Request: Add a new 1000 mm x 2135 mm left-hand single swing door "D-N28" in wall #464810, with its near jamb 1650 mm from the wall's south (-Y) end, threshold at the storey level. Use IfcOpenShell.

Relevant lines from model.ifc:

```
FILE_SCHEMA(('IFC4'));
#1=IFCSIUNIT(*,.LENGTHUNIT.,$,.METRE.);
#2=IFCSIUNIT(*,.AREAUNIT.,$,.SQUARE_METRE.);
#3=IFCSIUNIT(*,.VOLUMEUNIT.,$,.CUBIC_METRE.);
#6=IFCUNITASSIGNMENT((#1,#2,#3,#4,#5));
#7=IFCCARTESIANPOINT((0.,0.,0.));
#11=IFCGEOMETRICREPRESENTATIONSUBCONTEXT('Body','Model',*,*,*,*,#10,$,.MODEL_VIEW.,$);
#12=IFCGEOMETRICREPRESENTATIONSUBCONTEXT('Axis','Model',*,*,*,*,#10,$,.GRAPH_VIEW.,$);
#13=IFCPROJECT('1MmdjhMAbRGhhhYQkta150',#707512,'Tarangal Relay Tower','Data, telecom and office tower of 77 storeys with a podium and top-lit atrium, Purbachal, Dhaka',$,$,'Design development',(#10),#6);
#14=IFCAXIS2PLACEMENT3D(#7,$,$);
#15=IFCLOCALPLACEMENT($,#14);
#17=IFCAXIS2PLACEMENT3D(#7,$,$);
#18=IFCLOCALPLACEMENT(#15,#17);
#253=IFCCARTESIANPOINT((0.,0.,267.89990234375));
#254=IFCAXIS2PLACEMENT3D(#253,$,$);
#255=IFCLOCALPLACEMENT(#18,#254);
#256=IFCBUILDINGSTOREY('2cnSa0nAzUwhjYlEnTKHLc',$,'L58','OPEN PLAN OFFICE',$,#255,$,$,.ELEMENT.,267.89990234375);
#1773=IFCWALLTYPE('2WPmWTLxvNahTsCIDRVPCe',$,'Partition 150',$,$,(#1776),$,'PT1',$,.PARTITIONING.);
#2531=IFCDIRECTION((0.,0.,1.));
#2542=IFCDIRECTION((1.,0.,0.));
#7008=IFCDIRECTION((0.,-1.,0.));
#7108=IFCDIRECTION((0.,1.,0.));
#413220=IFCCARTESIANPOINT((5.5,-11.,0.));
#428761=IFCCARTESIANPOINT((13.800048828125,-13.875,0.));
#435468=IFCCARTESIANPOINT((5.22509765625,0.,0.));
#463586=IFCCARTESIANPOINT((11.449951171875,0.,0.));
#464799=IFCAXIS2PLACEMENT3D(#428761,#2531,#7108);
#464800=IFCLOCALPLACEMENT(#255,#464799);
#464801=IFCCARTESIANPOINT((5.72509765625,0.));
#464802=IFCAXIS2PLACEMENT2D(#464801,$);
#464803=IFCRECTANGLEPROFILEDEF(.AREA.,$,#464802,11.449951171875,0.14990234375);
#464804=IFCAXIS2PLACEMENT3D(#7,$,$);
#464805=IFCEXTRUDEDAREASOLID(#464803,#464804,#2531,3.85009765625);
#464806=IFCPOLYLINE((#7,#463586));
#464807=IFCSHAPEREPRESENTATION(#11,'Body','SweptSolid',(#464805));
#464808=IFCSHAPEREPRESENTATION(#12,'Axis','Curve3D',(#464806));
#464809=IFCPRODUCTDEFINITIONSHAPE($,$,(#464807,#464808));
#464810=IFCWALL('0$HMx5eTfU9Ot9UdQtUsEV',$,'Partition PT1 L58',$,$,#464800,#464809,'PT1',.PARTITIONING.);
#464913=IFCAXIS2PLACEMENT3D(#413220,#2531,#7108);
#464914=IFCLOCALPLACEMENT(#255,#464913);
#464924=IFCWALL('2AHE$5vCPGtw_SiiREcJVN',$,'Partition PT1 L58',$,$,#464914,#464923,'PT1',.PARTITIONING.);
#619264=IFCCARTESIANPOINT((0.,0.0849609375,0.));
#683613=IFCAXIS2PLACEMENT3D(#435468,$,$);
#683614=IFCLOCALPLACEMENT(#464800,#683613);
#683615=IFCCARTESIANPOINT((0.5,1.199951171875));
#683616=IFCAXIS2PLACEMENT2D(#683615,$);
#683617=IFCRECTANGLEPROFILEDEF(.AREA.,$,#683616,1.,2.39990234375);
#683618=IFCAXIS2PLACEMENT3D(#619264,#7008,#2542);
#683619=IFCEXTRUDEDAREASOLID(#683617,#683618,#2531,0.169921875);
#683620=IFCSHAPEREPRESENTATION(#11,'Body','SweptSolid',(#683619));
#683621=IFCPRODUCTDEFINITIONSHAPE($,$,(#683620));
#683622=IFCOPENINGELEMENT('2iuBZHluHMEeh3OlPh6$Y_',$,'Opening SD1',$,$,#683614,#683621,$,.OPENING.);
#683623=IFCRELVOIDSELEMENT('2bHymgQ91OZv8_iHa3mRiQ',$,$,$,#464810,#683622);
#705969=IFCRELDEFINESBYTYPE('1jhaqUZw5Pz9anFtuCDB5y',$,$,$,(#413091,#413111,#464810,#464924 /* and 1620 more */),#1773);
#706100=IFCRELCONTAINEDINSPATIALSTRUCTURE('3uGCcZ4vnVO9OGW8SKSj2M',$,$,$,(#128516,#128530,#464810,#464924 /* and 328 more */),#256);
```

```python
import numpy as np
import ifcopenshell
import ifcopenshell.api.feature
import ifcopenshell.api.geometry
import ifcopenshell.api.root
import ifcopenshell.api.spatial
import ifcopenshell.geom
import ifcopenshell.util.element
import ifcopenshell.util.placement
import ifcopenshell.util.representation
import ifcopenshell.util.shape
import ifcopenshell.util.unit

model = ifcopenshell.open("model.ifc")
unit_scale = ifcopenshell.util.unit.calculate_unit_scale(model)
settings = ifcopenshell.geom.settings()


def volume(element):
    """Net volume in cubic metres, openings subtracted."""
    shape = ifcopenshell.geom.create_shape(settings, element)
    return ifcopenshell.util.shape.get_volume(shape.geometry)


wall = model.by_id(464810)
storey = ifcopenshell.util.element.get_container(wall, ifc_class="IfcBuildingStorey")
context = ifcopenshell.util.representation.get_context(model, "Model", "Body", "MODEL_VIEW")
before = volume(wall)

width, height, from_end, sill = 1, 2.135, 1.65, 0.0  # metres

# The wall runs along its own X axis, and the end named is its -X end.
wall_shape = ifcopenshell.geom.create_shape(settings, wall)
x, y, z = ifcopenshell.util.shape.get_vertices(wall_shape.geometry).T
start = x.min() + from_end
face, thickness = float(y.min()), float(y.max() - y.min())
wall_matrix = ifcopenshell.util.placement.get_local_placement(wall.ObjectPlacement)
level = ifcopenshell.util.placement.get_local_placement(storey.ObjectPlacement)[2, 3]


def in_wall(x, y):
    """Placement at x, y metres in the wall's axes, at sill height."""
    matrix = wall_matrix.copy()
    matrix[:, 3] = wall_matrix @ np.array([x / unit_scale, y / unit_scale, 0.0, 1.0])
    matrix[2, 3] = level + sill / unit_scale
    return matrix


# Opening: a box that overshoots both wall faces by 50 mm.
opening = ifcopenshell.api.root.create_entity(model, ifc_class="IfcOpeningElement", predefined_type="OPENING")
box = ifcopenshell.api.geometry.add_wall_representation(
    model, context=context, length=width, height=height, thickness=thickness + 0.1
)
ifcopenshell.api.geometry.assign_representation(model, product=opening, representation=box)
ifcopenshell.api.geometry.edit_object_placement(model, product=opening, matrix=in_wall(start, face - 0.05), is_si=False)
ifcopenshell.api.feature.add_feature(model, feature=opening, element=wall)

door = ifcopenshell.api.root.create_entity(model, ifc_class="IfcDoor", name="D-N28", predefined_type="DOOR")
door.OverallWidth, door.OverallHeight = width / unit_scale, height / unit_scale
door.OperationType = "SINGLE_SWING_LEFT"
body = ifcopenshell.api.geometry.add_door_representation(
    model,
    context=context,
    overall_width=door.OverallWidth,
    overall_height=door.OverallHeight,
    operation_type="SINGLE_SWING_LEFT",
    lining_properties={"LiningDepth": thickness / unit_scale, "ThresholdDepth": thickness / unit_scale},
)
ifcopenshell.api.geometry.assign_representation(model, product=door, representation=body)
ifcopenshell.api.spatial.assign_container(model, products=[door], relating_structure=storey)
ifcopenshell.api.feature.add_filling(model, opening=opening, element=door)

# The lining spans the wall, so the door starts at the wall face.
ifcopenshell.api.geometry.edit_object_placement(model, product=door, matrix=in_wall(start, face), is_si=False)

after = volume(wall)

print(f"wall volume {before:.3f} -> {after:.3f} m3")

model.write("model_rev.ifc")
```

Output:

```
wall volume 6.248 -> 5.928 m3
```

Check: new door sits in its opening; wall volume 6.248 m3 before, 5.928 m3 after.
